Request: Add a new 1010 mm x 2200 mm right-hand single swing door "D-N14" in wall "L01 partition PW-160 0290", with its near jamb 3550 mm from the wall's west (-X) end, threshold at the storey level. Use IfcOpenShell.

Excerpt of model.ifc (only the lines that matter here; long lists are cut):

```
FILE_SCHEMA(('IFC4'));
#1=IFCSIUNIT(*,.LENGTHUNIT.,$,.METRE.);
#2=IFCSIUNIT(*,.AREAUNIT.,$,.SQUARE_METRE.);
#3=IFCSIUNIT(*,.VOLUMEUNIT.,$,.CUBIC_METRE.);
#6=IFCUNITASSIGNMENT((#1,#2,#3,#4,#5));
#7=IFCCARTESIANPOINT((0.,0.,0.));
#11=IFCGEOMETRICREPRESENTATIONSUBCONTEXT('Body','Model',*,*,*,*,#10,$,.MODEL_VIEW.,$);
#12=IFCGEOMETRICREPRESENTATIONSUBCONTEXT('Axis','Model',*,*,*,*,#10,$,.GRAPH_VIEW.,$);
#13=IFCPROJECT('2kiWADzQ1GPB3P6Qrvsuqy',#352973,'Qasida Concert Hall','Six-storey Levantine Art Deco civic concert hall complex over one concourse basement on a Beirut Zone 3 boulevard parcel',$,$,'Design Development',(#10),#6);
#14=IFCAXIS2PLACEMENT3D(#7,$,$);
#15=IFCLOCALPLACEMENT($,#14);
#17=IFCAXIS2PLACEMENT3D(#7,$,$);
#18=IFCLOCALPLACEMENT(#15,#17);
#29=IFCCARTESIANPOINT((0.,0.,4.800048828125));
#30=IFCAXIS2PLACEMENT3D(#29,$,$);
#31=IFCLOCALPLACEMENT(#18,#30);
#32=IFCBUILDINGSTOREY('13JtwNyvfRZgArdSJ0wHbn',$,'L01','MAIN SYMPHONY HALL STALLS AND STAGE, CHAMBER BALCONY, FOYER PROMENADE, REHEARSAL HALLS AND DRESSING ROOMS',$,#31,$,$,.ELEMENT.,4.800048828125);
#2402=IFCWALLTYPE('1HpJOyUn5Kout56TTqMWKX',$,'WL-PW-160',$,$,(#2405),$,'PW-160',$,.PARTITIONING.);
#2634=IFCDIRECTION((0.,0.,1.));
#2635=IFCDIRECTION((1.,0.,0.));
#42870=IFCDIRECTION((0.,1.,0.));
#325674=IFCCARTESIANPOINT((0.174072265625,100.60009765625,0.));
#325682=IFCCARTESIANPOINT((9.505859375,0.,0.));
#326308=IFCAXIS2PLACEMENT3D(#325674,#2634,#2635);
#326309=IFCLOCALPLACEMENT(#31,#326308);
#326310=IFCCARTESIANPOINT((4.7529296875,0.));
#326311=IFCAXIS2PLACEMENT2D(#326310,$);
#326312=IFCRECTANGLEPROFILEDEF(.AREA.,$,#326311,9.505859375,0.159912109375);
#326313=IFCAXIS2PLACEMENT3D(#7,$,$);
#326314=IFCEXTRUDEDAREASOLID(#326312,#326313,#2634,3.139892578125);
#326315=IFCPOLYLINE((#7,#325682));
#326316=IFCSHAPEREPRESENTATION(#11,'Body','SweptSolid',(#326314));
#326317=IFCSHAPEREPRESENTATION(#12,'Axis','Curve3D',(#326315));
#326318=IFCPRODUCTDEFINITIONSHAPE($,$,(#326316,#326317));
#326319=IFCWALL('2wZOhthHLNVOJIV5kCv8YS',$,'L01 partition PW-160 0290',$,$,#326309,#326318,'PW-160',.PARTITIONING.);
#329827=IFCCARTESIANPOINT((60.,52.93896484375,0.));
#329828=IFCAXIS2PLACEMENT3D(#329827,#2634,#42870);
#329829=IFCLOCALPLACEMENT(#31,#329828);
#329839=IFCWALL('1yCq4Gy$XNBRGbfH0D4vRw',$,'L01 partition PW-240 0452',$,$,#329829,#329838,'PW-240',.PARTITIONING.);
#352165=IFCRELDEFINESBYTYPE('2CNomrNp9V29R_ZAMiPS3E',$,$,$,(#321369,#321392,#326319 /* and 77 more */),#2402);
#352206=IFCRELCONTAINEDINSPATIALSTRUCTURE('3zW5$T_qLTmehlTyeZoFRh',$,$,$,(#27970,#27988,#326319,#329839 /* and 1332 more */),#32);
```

```python
import numpy as np
import ifcopenshell
import ifcopenshell.api.feature
import ifcopenshell.api.geometry
import ifcopenshell.api.root
import ifcopenshell.api.spatial
import ifcopenshell.geom
import ifcopenshell.util.element
import ifcopenshell.util.placement
import ifcopenshell.util.representation
import ifcopenshell.util.shape
import ifcopenshell.util.unit

model = ifcopenshell.open("model.ifc")
unit_scale = ifcopenshell.util.unit.calculate_unit_scale(model)
settings = ifcopenshell.geom.settings()


def volume(element):
    """Net volume in cubic metres, openings subtracted."""
    shape = ifcopenshell.geom.create_shape(settings, element)
    return ifcopenshell.util.shape.get_volume(shape.geometry)


wall = model.by_id(326319)
storey = ifcopenshell.util.element.get_container(wall, ifc_class="IfcBuildingStorey")
context = ifcopenshell.util.representation.get_context(model, "Model", "Body", "MODEL_VIEW")
before = volume(wall)

width, height, from_end, sill = 1.01, 2.2, 3.55, 0.0  # metres

# The wall runs along its own X axis, and the end named is its -X end.
wall_shape = ifcopenshell.geom.create_shape(settings, wall)
x, y, z = ifcopenshell.util.shape.get_vertices(wall_shape.geometry).T
start = x.min() + from_end
face, thickness = float(y.min()), float(y.max() - y.min())
wall_matrix = ifcopenshell.util.placement.get_local_placement(wall.ObjectPlacement)
level = ifcopenshell.util.placement.get_local_placement(storey.ObjectPlacement)[2, 3]


def in_wall(x, y):
    """Placement at x, y metres in the wall's axes, at sill height."""
    matrix = wall_matrix.copy()
    matrix[:, 3] = wall_matrix @ np.array([x / unit_scale, y / unit_scale, 0.0, 1.0])
    matrix[2, 3] = level + sill / unit_scale
    return matrix


# Opening: a box that overshoots both wall faces by 50 mm.
opening = ifcopenshell.api.root.create_entity(model, ifc_class="IfcOpeningElement", predefined_type="OPENING")
box = ifcopenshell.api.geometry.add_wall_representation(
    model, context=context, length=width, height=height, thickness=thickness + 0.1
)
ifcopenshell.api.geometry.assign_representation(model, product=opening, representation=box)
ifcopenshell.api.geometry.edit_object_placement(model, product=opening, matrix=in_wall(start, face - 0.05), is_si=False)
ifcopenshell.api.feature.add_feature(model, feature=opening, element=wall)

door = ifcopenshell.api.root.create_entity(model, ifc_class="IfcDoor", name="D-N14", predefined_type="DOOR")
door.OverallWidth, door.OverallHeight = width / unit_scale, height / unit_scale
door.OperationType = "SINGLE_SWING_RIGHT"
body = ifcopenshell.api.geometry.add_door_representation(
    model,
    context=context,
    overall_width=door.OverallWidth,
    overall_height=door.OverallHeight,
    operation_type="SINGLE_SWING_RIGHT",
    lining_properties={"LiningDepth": thickness / unit_scale, "ThresholdDepth": thickness / unit_scale},
)
ifcopenshell.api.geometry.assign_representation(model, product=door, representation=body)
ifcopenshell.api.spatial.assign_container(model, products=[door], relating_structure=storey)
ifcopenshell.api.feature.add_filling(model, opening=opening, element=door)

# The lining spans the wall, so the door starts at the wall face.
ifcopenshell.api.geometry.edit_object_placement(model, product=door, matrix=in_wall(start, face), is_si=False)

after = volume(wall)

print(f"wall volume {before:.3f} -> {after:.3f} m3")

model.write("model-out.ifc")
```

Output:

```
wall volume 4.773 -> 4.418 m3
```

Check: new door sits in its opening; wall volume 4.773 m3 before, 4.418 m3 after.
